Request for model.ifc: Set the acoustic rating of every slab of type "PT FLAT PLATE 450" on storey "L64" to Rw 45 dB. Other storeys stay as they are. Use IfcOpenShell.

First a look at what the model holds.

```python
import ifcopenshell
import ifcopenshell.util.element

model = ifcopenshell.open("model.ifc")
print(model.schema)
storey = next(s for s in model.by_type("IfcBuildingStorey") if s.Name == "L64")
slabs = [e for e in ifcopenshell.util.element.get_decomposition(storey) if e.is_a("IfcSlab")]
seen = {}
for e in slabs:
    element_type = ifcopenshell.util.element.get_type(e)
    key = (element_type.Name if element_type != e and element_type else None, ifcopenshell.util.element.get_pset(e, "Pset_SlabCommon", "AcousticRating"))
    seen[key] = seen.get(key, 0) + 1
for (name, value), count in sorted(seen.items(), key=str):
    print(count, "x", name, "|", value)
```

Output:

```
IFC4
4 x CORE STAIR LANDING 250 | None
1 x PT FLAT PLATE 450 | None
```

```python
import ifcopenshell
import ifcopenshell.api.pset
import ifcopenshell.util.element

model = ifcopenshell.open("model.ifc")

storey = next(s for s in model.by_type("IfcBuildingStorey") if s.Name == "L64")
slabs = [e for e in ifcopenshell.util.element.get_decomposition(storey) if e.is_a("IfcSlab")]

count = 0
for e in slabs:
    element_type = ifcopenshell.util.element.get_type(e)
    if element_type in (None, e) or element_type.Name != "PT FLAT PLATE 450":
        continue
    found = ifcopenshell.util.element.get_pset(e, "Pset_SlabCommon", should_inherit=False)
    if found:
        pset = model.by_id(found["id"])
        if len(ifcopenshell.util.element.get_elements_by_pset(pset)) > 1:
            pset = ifcopenshell.api.pset.unshare_pset(model, products=[e], pset=pset)[0]
    else:
        pset = ifcopenshell.api.pset.add_pset(model, product=e, name="Pset_SlabCommon")
    ifcopenshell.api.pset.edit_pset(model, pset=pset, properties={"AcousticRating": "Rw 45 dB"})
    count += 1

print(count, "slabs updated")

model.write("model_updated.ifc")
```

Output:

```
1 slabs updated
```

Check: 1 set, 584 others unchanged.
